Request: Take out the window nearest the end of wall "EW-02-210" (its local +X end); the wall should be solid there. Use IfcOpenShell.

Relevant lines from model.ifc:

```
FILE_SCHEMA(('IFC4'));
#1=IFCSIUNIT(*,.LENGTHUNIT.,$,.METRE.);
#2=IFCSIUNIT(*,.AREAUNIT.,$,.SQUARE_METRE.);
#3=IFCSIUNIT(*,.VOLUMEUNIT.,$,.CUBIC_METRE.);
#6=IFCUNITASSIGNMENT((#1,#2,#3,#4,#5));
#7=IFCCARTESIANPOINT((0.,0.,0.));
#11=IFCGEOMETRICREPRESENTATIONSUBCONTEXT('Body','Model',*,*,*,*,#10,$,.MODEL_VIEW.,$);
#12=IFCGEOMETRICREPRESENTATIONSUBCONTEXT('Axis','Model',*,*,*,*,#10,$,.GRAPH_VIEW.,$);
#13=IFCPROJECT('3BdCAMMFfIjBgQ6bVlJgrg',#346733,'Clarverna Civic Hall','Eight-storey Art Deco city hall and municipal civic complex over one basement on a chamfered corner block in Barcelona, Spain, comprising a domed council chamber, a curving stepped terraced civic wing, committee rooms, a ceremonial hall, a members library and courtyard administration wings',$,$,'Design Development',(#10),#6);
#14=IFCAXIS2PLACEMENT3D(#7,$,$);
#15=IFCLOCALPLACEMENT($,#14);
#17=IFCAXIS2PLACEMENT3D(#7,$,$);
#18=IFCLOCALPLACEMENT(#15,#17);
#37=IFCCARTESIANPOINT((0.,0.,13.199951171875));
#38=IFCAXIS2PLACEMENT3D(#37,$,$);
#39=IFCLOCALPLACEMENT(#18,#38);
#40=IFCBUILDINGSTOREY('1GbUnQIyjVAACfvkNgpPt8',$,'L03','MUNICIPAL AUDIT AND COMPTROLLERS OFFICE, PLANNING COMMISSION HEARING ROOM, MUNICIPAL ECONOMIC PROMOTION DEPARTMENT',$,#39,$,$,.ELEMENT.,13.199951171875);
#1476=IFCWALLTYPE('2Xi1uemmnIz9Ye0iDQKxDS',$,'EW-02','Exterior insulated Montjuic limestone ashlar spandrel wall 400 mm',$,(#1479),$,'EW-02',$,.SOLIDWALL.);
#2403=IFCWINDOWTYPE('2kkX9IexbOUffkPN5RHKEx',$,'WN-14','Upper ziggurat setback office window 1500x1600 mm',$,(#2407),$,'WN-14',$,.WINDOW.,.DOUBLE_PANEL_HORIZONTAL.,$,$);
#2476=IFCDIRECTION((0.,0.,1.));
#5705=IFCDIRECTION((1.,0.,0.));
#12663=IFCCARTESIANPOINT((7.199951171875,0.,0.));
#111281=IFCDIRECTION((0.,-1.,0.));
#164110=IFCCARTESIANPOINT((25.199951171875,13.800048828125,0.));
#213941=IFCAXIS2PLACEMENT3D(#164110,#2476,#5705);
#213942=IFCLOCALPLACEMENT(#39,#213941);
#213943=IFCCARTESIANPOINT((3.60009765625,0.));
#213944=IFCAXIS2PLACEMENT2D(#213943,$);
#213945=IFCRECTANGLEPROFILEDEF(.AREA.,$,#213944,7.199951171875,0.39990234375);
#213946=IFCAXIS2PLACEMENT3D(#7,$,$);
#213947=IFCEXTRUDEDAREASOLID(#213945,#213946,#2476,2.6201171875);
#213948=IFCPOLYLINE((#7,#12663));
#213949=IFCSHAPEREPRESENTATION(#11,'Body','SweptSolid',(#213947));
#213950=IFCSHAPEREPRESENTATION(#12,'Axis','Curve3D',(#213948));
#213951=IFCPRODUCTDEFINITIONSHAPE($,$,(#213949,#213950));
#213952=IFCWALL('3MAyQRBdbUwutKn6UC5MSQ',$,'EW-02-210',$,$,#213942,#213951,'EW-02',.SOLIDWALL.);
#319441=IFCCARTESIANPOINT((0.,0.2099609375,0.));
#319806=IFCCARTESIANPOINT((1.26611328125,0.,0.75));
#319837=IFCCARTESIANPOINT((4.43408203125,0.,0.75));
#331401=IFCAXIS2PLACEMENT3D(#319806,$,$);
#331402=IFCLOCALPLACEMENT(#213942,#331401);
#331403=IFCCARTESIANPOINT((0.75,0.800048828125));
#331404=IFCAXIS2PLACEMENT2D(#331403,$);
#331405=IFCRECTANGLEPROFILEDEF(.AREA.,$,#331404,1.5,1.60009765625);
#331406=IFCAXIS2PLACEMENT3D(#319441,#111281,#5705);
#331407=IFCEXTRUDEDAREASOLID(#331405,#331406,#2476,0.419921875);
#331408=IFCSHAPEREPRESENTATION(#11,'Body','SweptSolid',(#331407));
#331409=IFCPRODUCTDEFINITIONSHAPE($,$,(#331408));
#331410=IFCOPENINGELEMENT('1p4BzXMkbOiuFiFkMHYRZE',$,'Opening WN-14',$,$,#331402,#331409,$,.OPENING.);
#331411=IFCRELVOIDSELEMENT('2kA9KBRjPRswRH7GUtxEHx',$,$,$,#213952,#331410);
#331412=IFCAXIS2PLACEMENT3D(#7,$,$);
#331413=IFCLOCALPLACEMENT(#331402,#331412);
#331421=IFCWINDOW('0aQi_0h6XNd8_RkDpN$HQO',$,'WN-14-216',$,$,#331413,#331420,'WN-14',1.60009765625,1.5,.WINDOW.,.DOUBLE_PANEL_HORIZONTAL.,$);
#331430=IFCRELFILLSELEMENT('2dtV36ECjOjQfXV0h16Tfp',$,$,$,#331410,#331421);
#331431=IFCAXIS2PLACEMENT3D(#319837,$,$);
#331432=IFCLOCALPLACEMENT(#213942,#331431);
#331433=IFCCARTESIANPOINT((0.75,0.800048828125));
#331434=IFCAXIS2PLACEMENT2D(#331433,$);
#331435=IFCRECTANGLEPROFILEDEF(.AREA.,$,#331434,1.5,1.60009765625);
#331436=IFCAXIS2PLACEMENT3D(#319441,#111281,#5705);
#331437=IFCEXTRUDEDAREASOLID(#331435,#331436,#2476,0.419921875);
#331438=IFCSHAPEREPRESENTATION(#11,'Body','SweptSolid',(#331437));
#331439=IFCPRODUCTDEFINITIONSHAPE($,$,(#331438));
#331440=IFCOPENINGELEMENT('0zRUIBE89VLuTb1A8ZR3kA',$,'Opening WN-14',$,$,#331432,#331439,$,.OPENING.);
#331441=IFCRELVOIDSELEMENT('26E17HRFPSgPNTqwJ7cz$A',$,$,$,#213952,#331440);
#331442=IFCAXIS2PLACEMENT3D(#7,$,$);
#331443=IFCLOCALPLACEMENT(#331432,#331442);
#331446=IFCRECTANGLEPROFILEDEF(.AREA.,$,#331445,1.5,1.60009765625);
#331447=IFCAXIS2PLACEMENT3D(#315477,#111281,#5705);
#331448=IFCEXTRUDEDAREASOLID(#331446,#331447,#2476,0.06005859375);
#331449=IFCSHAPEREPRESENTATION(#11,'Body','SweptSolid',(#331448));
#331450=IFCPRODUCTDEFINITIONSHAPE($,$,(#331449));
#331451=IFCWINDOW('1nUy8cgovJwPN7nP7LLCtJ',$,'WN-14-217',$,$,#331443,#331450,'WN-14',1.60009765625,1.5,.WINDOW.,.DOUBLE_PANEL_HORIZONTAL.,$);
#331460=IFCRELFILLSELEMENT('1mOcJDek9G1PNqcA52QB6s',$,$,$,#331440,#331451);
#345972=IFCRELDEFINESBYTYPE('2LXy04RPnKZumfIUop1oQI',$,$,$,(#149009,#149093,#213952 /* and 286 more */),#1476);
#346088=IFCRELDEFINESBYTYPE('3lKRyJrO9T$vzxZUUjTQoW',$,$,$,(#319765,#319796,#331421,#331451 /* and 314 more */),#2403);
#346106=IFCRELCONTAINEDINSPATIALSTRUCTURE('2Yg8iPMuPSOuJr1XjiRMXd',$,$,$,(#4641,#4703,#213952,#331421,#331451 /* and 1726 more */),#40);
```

```python
import ifcopenshell
import ifcopenshell.api.feature
import ifcopenshell.api.root
import ifcopenshell.geom
import ifcopenshell.util.shape

model = ifcopenshell.open("model.ifc")
settings = ifcopenshell.geom.settings()


def volume(element):
    """Net volume in cubic metres, openings subtracted."""
    shape = ifcopenshell.geom.create_shape(settings, element)
    return ifcopenshell.util.shape.get_volume(shape.geometry)


window = model.by_guid("1nUy8cgovJwPN7nP7LLCtJ")
opening = window.FillsVoids[0].RelatingOpeningElement
wall = opening.VoidsElements[0].RelatingBuildingElement
before = volume(wall)

ifcopenshell.api.root.remove_product(model, product=window)
ifcopenshell.api.feature.remove_feature(model, feature=opening)

after = volume(wall)

print(f"wall volume {before:.3f} -> {after:.3f} m3")

model.write("model_updated.ifc")
```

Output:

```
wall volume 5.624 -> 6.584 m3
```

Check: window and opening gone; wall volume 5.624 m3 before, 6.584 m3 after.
